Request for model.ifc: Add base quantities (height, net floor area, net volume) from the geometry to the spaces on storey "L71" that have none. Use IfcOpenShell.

First a look at what the model holds.

```python
import ifcopenshell
import ifcopenshell.util.element
import ifcopenshell.util.unit

model = ifcopenshell.open("model.ifc")
print(model.schema)
for unit_type in ("LENGTHUNIT", "AREAUNIT", "VOLUMEUNIT"):
    print(unit_type, ifcopenshell.util.unit.calculate_unit_scale(model, unit_type))
storey = next(s for s in model.by_type("IfcBuildingStorey") if s.Name == "L71")
spaces = [e for e in ifcopenshell.util.element.get_decomposition(storey) if e.is_a("IfcSpace")]
for e in sorted(spaces, key=lambda e: e.id()):
    print(e.id(), e.is_a(), e.Name, list(ifcopenshell.util.element.get_psets(e, qtos_only=True)), sep=" | ")
```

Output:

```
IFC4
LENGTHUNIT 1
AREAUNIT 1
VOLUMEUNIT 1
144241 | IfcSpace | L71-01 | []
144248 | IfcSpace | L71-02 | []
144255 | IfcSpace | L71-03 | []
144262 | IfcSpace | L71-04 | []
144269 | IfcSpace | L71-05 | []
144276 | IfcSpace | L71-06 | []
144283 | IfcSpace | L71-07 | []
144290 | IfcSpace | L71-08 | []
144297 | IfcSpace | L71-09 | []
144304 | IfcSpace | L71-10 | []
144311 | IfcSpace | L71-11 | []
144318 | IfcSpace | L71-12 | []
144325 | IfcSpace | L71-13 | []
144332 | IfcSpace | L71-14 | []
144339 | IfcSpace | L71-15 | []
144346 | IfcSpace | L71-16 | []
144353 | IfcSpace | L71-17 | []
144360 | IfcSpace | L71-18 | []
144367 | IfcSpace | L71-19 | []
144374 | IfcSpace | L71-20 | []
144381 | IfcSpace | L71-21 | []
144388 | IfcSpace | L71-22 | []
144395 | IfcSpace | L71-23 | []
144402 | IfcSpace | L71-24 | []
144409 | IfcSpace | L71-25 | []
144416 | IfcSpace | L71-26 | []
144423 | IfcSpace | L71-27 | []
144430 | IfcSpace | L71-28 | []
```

```python
import ifcopenshell
import ifcopenshell.api.pset
import ifcopenshell.geom
import ifcopenshell.util.element
import ifcopenshell.util.shape
import ifcopenshell.util.unit

model = ifcopenshell.open("model.ifc")
unit_scale = ifcopenshell.util.unit.calculate_unit_scale(model)
area_scale = ifcopenshell.util.unit.calculate_unit_scale(model, "AREAUNIT")
volume_scale = ifcopenshell.util.unit.calculate_unit_scale(model, "VOLUMEUNIT")
settings = ifcopenshell.geom.settings()

storey = next(s for s in model.by_type("IfcBuildingStorey") if s.Name == "L71")
spaces = [e for e in ifcopenshell.util.element.get_decomposition(storey) if e.is_a("IfcSpace")]

for e in sorted(spaces, key=lambda e: e.id()):
    if ifcopenshell.util.element.get_psets(e, qtos_only=True, should_inherit=False):
        continue
    # Geometry comes back in metres, in the element's own axes.
    shape = ifcopenshell.geom.create_shape(settings, e)
    values = {
        "Height": ifcopenshell.util.shape.get_z(shape.geometry) / unit_scale,
        "NetFloorArea": ifcopenshell.util.shape.get_footprint_area(shape.geometry) / area_scale,
        "NetVolume": ifcopenshell.util.shape.get_volume(shape.geometry) / volume_scale,
    }
    qto = ifcopenshell.api.pset.add_qto(model, product=e, name="Qto_SpaceBaseQuantities")
    ifcopenshell.api.pset.edit_qto(model, qto=qto, properties=values)
    print(e.id(), {k: round(v, 3) for k, v in values.items()})

model.write("model_edited.ifc")
```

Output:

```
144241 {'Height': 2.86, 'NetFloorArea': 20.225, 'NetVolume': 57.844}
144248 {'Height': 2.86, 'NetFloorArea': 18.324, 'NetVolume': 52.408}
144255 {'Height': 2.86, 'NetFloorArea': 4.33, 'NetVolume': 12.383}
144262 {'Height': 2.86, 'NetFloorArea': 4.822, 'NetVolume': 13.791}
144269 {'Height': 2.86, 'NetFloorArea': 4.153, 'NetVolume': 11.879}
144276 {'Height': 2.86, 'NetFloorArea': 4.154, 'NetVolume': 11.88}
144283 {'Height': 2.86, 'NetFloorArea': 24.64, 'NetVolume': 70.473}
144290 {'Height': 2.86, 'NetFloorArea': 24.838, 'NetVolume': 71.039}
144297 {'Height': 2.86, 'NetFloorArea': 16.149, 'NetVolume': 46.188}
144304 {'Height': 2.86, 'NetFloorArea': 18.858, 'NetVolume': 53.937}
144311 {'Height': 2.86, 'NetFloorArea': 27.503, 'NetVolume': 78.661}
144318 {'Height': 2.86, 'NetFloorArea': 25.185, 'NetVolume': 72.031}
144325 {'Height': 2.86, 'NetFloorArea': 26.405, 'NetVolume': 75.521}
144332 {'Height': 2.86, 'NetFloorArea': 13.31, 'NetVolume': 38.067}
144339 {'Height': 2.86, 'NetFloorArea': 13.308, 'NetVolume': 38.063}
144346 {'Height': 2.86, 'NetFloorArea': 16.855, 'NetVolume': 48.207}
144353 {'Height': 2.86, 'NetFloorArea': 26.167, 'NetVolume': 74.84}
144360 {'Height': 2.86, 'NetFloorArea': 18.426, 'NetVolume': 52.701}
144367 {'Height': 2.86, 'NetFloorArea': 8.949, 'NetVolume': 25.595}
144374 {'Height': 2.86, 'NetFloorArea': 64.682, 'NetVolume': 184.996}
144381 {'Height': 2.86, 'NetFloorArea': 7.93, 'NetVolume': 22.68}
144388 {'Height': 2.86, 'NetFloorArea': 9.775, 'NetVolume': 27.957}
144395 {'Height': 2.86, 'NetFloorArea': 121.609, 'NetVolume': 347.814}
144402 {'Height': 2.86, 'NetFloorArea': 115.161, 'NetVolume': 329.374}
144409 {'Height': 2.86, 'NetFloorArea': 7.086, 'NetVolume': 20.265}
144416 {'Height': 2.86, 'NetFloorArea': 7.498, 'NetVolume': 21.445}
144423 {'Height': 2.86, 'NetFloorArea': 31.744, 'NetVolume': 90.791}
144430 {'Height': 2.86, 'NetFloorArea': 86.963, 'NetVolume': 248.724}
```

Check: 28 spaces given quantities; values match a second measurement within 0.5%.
